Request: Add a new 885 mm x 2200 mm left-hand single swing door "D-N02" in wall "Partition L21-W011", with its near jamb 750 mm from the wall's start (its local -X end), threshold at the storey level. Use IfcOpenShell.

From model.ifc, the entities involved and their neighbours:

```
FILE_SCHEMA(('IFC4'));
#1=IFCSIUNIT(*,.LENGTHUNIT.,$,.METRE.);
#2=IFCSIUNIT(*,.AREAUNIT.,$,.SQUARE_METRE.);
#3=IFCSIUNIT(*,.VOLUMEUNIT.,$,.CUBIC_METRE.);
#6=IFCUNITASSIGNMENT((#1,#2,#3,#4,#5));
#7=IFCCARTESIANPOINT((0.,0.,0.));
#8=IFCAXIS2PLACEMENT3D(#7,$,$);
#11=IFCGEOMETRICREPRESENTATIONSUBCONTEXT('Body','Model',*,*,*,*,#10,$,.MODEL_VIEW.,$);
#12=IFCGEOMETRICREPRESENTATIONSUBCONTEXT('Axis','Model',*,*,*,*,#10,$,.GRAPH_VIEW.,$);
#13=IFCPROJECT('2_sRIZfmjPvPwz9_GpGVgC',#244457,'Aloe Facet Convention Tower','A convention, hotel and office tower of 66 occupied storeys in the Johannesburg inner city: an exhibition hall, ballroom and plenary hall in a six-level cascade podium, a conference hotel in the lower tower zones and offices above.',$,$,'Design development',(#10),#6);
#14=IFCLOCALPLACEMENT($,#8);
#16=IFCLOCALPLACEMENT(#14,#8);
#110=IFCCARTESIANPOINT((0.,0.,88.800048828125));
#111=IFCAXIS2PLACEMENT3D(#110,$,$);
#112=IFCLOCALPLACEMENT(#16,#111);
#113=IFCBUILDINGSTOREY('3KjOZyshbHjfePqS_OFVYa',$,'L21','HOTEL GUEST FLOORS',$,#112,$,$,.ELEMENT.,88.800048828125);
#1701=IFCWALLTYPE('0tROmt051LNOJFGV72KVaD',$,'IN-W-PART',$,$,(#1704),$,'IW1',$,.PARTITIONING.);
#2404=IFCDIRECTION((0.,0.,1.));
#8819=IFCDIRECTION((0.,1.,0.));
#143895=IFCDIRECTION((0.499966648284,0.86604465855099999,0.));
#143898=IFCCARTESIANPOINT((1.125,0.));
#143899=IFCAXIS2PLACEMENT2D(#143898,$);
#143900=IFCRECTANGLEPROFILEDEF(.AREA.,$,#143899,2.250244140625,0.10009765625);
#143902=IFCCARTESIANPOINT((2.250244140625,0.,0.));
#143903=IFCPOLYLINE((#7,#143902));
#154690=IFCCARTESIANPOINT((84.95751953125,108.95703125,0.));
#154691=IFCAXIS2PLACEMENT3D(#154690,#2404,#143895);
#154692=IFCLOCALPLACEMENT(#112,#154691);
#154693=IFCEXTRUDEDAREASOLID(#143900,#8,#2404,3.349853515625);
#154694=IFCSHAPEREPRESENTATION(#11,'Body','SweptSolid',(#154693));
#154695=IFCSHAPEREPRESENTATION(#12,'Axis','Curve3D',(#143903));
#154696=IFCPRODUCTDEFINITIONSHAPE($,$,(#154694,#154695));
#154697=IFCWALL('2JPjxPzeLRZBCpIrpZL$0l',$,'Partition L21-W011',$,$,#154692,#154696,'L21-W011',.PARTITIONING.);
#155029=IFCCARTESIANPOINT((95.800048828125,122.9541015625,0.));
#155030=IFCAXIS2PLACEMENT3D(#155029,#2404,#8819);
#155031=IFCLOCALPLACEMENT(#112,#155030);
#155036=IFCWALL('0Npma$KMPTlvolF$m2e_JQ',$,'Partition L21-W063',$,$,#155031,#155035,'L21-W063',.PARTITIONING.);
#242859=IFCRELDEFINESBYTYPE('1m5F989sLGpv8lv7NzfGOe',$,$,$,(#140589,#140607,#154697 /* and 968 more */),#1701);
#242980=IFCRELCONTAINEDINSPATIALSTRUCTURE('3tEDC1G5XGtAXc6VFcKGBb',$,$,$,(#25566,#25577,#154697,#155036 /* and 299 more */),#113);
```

```python
import numpy as np
import ifcopenshell
import ifcopenshell.api.feature
import ifcopenshell.api.geometry
import ifcopenshell.api.root
import ifcopenshell.api.spatial
import ifcopenshell.geom
import ifcopenshell.util.element
import ifcopenshell.util.placement
import ifcopenshell.util.representation
import ifcopenshell.util.shape
import ifcopenshell.util.unit

model = ifcopenshell.open("model.ifc")
unit_scale = ifcopenshell.util.unit.calculate_unit_scale(model)
settings = ifcopenshell.geom.settings()


def volume(element):
    """Net volume in cubic metres, openings subtracted."""
    shape = ifcopenshell.geom.create_shape(settings, element)
    return ifcopenshell.util.shape.get_volume(shape.geometry)


wall = model.by_guid("2JPjxPzeLRZBCpIrpZL$0l")
storey = ifcopenshell.util.element.get_container(wall, ifc_class="IfcBuildingStorey")
context = ifcopenshell.util.representation.get_context(model, "Model", "Body", "MODEL_VIEW")
before = volume(wall)

width, height, from_end, sill = 0.885, 2.2, 0.75, 0.0  # metres

# The wall runs along its own X axis, and the end named is its -X end.
wall_shape = ifcopenshell.geom.create_shape(settings, wall)
x, y, z = ifcopenshell.util.shape.get_vertices(wall_shape.geometry).T
start = x.min() + from_end
face, thickness = float(y.min()), float(y.max() - y.min())
wall_matrix = ifcopenshell.util.placement.get_local_placement(wall.ObjectPlacement)
level = ifcopenshell.util.placement.get_local_placement(storey.ObjectPlacement)[2, 3]


def in_wall(x, y):
    """Placement at x, y metres in the wall's axes, at sill height."""
    matrix = wall_matrix.copy()
    matrix[:, 3] = wall_matrix @ np.array([x / unit_scale, y / unit_scale, 0.0, 1.0])
    matrix[2, 3] = level + sill / unit_scale
    return matrix


# Opening: a box that overshoots both wall faces by 50 mm.
opening = ifcopenshell.api.root.create_entity(model, ifc_class="IfcOpeningElement", predefined_type="OPENING")
box = ifcopenshell.api.geometry.add_wall_representation(
    model, context=context, length=width, height=height, thickness=thickness + 0.1
)
ifcopenshell.api.geometry.assign_representation(model, product=opening, representation=box)
ifcopenshell.api.geometry.edit_object_placement(model, product=opening, matrix=in_wall(start, face - 0.05), is_si=False)
ifcopenshell.api.feature.add_feature(model, feature=opening, element=wall)

door = ifcopenshell.api.root.create_entity(model, ifc_class="IfcDoor", name="D-N02", predefined_type="DOOR")
door.OverallWidth, door.OverallHeight = width / unit_scale, height / unit_scale
door.OperationType = "SINGLE_SWING_LEFT"
body = ifcopenshell.api.geometry.add_door_representation(
    model,
    context=context,
    overall_width=door.OverallWidth,
    overall_height=door.OverallHeight,
    operation_type="SINGLE_SWING_LEFT",
    lining_properties={"LiningDepth": thickness / unit_scale, "ThresholdDepth": thickness / unit_scale},
)
ifcopenshell.api.geometry.assign_representation(model, product=door, representation=body)
ifcopenshell.api.spatial.assign_container(model, products=[door], relating_structure=storey)
ifcopenshell.api.feature.add_filling(model, opening=opening, element=door)

# The lining spans the wall, so the door starts at the wall face.
ifcopenshell.api.geometry.edit_object_placement(model, product=door, matrix=in_wall(start, face), is_si=False)

after = volume(wall)

print(f"wall volume {before:.3f} -> {after:.3f} m3")

model.write("model-out.ifc")
```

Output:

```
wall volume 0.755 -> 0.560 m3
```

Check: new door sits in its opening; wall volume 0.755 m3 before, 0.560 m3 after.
